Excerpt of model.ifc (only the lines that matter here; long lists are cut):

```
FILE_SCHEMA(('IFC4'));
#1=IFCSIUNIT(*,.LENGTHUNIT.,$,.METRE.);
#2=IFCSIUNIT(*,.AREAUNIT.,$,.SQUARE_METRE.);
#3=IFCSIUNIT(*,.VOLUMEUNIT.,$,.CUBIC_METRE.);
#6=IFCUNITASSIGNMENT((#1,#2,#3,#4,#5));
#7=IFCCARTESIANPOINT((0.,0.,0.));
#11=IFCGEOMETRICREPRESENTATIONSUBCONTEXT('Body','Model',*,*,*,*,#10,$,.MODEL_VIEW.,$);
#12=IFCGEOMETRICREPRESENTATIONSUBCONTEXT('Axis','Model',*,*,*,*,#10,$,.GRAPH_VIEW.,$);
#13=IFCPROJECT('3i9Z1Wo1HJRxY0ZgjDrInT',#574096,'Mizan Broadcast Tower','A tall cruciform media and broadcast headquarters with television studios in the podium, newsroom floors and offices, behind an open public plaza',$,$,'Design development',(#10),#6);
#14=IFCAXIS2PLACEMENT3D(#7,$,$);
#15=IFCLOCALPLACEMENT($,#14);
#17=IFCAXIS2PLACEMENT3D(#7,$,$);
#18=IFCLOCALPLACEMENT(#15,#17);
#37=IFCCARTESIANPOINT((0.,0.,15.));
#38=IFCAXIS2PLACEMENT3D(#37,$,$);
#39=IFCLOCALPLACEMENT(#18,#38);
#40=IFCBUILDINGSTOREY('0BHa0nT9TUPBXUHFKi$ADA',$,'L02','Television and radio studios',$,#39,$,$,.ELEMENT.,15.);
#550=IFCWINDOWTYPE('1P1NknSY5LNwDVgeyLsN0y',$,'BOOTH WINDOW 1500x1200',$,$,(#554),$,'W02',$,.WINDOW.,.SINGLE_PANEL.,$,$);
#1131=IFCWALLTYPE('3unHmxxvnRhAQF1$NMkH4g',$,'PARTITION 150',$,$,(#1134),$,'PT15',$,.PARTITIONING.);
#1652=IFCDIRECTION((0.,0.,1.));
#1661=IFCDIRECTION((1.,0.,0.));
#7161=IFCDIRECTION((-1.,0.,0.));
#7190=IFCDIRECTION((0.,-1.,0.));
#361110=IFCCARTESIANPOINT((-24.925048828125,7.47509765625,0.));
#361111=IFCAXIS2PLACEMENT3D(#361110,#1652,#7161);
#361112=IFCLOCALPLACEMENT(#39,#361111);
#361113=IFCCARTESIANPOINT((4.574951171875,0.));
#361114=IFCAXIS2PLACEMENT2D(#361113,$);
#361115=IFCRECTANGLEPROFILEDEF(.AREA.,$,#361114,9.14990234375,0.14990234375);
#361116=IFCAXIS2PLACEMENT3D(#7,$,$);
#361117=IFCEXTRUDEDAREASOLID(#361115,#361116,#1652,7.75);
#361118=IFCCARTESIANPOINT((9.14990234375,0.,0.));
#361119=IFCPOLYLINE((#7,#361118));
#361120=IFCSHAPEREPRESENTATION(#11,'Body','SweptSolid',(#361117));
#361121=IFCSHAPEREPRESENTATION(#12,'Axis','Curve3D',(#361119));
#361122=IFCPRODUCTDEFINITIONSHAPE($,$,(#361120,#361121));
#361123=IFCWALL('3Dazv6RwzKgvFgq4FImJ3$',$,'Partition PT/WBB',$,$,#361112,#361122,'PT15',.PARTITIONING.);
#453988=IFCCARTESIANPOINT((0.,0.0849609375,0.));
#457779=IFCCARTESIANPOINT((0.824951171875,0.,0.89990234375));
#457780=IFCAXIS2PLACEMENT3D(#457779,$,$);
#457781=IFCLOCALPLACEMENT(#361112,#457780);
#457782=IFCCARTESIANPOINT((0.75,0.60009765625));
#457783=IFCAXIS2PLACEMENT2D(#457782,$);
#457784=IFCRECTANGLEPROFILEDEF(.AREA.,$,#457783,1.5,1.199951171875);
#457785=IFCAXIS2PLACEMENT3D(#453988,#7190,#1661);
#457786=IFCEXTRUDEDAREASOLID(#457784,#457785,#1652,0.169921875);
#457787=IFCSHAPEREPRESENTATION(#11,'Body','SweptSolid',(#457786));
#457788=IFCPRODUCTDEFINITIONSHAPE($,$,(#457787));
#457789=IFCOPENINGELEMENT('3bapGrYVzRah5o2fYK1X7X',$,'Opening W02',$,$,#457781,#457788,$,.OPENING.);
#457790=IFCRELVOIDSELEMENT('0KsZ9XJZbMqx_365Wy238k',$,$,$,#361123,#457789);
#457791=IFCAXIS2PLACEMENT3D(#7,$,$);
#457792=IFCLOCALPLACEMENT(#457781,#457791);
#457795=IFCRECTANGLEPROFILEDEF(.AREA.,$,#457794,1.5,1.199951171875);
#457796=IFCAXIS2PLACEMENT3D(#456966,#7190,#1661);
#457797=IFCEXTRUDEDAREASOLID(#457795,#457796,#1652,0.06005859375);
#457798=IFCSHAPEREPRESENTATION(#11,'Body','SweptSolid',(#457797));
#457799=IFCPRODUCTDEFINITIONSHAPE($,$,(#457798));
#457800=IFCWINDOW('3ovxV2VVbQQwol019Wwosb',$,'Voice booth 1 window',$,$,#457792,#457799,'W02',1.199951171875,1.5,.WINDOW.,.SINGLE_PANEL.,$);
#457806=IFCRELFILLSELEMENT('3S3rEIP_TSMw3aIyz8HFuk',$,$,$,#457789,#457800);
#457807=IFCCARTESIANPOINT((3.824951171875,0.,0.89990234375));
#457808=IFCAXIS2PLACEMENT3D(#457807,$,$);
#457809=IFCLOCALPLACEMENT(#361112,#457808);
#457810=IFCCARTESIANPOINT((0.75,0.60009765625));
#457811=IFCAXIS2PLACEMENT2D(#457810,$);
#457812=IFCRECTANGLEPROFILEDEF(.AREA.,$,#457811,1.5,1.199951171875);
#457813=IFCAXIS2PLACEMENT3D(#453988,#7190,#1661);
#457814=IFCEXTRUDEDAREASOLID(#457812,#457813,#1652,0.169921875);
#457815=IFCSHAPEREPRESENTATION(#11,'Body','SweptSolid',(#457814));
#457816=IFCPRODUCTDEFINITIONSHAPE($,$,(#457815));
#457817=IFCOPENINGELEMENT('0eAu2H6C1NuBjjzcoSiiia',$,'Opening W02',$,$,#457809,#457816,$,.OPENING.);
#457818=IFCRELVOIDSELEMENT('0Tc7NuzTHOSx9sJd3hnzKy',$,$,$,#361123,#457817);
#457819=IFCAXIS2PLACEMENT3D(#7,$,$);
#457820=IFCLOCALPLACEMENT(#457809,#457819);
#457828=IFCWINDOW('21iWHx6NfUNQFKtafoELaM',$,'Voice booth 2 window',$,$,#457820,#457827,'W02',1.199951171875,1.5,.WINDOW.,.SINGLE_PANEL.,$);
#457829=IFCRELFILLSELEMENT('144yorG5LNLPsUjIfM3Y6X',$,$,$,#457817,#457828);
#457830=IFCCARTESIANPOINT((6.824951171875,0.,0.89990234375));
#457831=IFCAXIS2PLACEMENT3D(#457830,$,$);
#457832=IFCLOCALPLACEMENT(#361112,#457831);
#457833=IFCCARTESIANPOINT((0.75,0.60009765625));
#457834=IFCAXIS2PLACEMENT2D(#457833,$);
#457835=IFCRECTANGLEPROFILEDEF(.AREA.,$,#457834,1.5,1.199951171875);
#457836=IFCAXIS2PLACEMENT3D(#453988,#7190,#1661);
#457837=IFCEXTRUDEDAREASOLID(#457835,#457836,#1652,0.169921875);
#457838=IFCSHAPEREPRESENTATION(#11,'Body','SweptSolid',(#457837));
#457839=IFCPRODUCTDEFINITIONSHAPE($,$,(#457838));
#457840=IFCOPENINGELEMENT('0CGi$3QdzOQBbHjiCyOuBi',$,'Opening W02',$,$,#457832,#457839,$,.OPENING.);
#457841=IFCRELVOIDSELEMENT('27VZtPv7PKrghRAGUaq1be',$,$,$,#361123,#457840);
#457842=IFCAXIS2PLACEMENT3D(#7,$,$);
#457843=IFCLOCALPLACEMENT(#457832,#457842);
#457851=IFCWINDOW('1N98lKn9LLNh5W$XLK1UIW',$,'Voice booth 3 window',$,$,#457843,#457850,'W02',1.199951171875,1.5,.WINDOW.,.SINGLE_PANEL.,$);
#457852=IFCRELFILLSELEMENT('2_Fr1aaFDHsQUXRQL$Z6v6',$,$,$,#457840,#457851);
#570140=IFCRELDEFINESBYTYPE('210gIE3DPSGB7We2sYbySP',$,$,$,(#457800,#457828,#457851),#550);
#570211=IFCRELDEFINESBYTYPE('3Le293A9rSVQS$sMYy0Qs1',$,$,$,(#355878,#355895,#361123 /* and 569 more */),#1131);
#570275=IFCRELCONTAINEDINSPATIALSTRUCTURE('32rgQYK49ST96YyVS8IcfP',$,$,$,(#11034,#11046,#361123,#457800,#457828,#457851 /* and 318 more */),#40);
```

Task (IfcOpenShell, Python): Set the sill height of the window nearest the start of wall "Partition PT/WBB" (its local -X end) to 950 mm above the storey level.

```python
import numpy as np
import ifcopenshell
import ifcopenshell.api.geometry
import ifcopenshell.geom
import ifcopenshell.util.element
import ifcopenshell.util.placement
import ifcopenshell.util.shape
import ifcopenshell.util.unit

model = ifcopenshell.open("model.ifc")
unit_scale = ifcopenshell.util.unit.calculate_unit_scale(model)

window = model.by_id(457800)
opening = window.FillsVoids[0].RelatingOpeningElement
storey = ifcopenshell.util.element.get_container(window, ifc_class="IfcBuildingStorey")
level = ifcopenshell.util.placement.get_local_placement(storey.ObjectPlacement)[2, 3]

# The opening's origin need not be at the sill, so measure its lowest point.
shape = ifcopenshell.geom.create_shape(ifcopenshell.geom.settings(), opening)
bottom = ifcopenshell.util.shape.get_shape_bottom_elevation(shape, shape.geometry) / unit_scale
dz = level + 0.95 - bottom

shift = np.array([0.0, 0.0, dz])
# The window is placed relative to its opening, so it follows when the opening moves.
matrix = ifcopenshell.util.placement.get_local_placement(opening.ObjectPlacement)
matrix[:3, 3] += shift
ifcopenshell.api.geometry.edit_object_placement(
    model, product=opening, matrix=matrix, is_si=False, should_transform_children=True
)

print(f"moved by {dz * unit_scale:+.3f} m")

model.write("model_v2.ifc")
```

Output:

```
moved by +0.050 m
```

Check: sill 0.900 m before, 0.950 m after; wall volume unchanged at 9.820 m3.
